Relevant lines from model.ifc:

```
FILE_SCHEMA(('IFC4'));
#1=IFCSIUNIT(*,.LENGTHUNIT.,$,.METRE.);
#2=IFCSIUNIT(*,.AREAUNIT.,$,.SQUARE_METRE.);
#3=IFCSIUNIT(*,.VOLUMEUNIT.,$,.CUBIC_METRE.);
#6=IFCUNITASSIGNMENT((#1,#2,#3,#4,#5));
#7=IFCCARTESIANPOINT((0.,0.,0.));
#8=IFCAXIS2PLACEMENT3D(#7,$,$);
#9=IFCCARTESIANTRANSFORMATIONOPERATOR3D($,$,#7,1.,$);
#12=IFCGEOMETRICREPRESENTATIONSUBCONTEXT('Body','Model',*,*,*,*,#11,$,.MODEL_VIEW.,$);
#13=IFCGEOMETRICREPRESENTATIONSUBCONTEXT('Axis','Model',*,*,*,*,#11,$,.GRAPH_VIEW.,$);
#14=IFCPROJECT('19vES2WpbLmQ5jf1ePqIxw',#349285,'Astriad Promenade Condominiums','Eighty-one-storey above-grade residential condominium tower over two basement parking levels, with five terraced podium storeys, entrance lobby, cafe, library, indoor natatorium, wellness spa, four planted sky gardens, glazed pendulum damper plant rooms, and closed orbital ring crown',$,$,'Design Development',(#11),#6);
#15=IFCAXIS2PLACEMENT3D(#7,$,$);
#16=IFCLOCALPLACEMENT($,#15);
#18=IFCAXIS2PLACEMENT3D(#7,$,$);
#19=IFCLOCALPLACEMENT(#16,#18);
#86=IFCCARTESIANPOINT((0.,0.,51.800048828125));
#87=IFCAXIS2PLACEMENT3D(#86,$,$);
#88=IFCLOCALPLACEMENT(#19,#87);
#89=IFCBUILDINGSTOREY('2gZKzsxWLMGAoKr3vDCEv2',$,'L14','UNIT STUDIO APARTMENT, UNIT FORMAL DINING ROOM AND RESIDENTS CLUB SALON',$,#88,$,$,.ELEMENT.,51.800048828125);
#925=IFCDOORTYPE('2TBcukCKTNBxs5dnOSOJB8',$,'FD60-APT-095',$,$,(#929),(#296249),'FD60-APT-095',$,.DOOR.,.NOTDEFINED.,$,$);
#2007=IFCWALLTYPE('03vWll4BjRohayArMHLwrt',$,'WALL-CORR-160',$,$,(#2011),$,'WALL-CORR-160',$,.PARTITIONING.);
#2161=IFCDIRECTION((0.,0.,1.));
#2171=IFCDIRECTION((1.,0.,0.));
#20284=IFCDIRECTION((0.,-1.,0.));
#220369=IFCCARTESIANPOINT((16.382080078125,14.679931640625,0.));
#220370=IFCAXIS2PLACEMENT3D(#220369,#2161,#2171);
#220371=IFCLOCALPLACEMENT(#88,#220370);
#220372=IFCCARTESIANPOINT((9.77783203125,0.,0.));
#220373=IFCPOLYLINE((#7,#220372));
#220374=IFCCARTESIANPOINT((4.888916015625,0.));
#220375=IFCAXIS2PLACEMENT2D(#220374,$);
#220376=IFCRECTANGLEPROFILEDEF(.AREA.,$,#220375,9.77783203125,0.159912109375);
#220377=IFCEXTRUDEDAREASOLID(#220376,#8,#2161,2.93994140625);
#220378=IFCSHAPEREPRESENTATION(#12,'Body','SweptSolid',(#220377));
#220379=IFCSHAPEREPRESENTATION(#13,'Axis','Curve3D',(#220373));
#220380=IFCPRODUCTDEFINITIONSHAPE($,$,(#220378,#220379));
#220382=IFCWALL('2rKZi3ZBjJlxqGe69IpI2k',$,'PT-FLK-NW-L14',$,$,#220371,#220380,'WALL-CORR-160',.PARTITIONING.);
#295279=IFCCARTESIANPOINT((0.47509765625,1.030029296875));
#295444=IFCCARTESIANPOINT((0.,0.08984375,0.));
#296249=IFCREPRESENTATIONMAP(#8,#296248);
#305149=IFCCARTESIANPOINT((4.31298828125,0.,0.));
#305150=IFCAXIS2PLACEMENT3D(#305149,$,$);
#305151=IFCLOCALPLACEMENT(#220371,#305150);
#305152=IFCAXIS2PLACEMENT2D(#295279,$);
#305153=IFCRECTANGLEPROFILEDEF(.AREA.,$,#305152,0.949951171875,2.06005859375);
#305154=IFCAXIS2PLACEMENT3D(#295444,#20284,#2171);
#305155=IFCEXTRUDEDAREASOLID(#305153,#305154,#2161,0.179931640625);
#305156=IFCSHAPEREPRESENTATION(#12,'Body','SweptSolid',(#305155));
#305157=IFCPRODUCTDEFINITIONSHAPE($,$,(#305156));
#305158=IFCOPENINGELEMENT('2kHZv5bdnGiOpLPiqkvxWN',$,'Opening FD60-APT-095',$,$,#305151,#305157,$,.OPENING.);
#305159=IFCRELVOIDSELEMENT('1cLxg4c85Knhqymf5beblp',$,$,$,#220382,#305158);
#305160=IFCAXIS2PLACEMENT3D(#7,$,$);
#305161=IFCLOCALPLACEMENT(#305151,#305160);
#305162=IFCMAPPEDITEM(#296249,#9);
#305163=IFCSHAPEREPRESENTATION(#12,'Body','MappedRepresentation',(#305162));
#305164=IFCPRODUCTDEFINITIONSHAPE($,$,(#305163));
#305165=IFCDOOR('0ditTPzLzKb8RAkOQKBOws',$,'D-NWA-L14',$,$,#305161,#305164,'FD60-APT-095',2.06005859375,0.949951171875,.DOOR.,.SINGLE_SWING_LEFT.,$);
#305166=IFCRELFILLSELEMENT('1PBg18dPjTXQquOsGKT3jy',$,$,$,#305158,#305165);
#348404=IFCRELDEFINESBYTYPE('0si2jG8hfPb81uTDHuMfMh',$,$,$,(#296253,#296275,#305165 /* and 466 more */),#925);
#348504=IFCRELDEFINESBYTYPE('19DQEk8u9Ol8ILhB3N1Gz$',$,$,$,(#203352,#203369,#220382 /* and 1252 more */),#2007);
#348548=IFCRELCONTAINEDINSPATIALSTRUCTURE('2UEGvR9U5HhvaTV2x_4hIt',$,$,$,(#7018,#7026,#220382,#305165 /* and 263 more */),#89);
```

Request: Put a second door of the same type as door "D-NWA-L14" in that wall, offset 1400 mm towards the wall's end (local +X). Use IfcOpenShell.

```python
import ifcopenshell
import ifcopenshell.api.feature
import ifcopenshell.api.geometry
import ifcopenshell.api.root
import ifcopenshell.geom
import ifcopenshell.util.element
import ifcopenshell.util.placement
import ifcopenshell.util.shape
import ifcopenshell.util.unit

model = ifcopenshell.open("model.ifc")
unit_scale = ifcopenshell.util.unit.calculate_unit_scale(model)
settings = ifcopenshell.geom.settings()


def volume(element):
    """Net volume in cubic metres, openings subtracted."""
    shape = ifcopenshell.geom.create_shape(settings, element)
    return ifcopenshell.util.shape.get_volume(shape.geometry)


door = model.by_id(305165)
opening = door.FillsVoids[0].RelatingOpeningElement
wall = opening.VoidsElements[0].RelatingBuildingElement
before = volume(wall)
shift = ifcopenshell.util.placement.get_local_placement(wall.ObjectPlacement)[:3, 0] * 1.4 / unit_scale

# copy_class copies the void relationship, type, container and properties, but no geometry.
new_opening = ifcopenshell.api.root.copy_class(model, product=opening)
new_opening.Representation = ifcopenshell.util.element.copy_deep(
    model, opening.Representation, exclude=["IfcGeometricRepresentationContext", "IfcRepresentationMap"]
)
new_door = ifcopenshell.api.root.copy_class(model, product=door)
new_door.Representation = ifcopenshell.util.element.copy_deep(
    model, door.Representation, exclude=["IfcGeometricRepresentationContext", "IfcRepresentationMap"]
)
new_door.Tag = None
ifcopenshell.api.feature.add_filling(model, opening=new_opening, element=new_door)

for old, new in ((opening, new_opening), (door, new_door)):
    matrix = ifcopenshell.util.placement.get_local_placement(old.ObjectPlacement)
    matrix[:3, 3] += shift
    ifcopenshell.api.geometry.edit_object_placement(model, product=new, matrix=matrix, is_si=False)

after = volume(wall)

print(f"wall volume {before:.3f} -> {after:.3f} m3")

model.write("model_updated.ifc")
```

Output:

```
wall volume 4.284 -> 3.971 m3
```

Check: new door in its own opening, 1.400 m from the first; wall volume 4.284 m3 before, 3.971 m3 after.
